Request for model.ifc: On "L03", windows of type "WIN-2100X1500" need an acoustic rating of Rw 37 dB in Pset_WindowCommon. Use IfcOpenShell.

First a look at what the model holds.

```python
import ifcopenshell
import ifcopenshell.util.element

model = ifcopenshell.open("model.ifc")
print(model.schema)
storey = next(s for s in model.by_type("IfcBuildingStorey") if s.Name == "L03")
windows = [e for e in ifcopenshell.util.element.get_decomposition(storey) if e.is_a("IfcWindow")]
seen = {}
for e in windows:
    element_type = ifcopenshell.util.element.get_type(e)
    key = (element_type.Name if element_type != e and element_type else None, ifcopenshell.util.element.get_pset(e, "Pset_WindowCommon", "AcousticRating"))
    seen[key] = seen.get(key, 0) + 1
for (name, value), count in sorted(seen.items(), key=str):
    print(count, "x", name, "|", value)
```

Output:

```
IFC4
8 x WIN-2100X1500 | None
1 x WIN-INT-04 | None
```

```python
import ifcopenshell
import ifcopenshell.api.pset
import ifcopenshell.util.element

model = ifcopenshell.open("model.ifc")

storey = next(s for s in model.by_type("IfcBuildingStorey") if s.Name == "L03")
windows = [e for e in ifcopenshell.util.element.get_decomposition(storey) if e.is_a("IfcWindow")]

count = 0
for e in windows:
    element_type = ifcopenshell.util.element.get_type(e)
    if element_type in (None, e) or element_type.Name != "WIN-2100X1500":
        continue
    # add_pset returns the element's existing set when there is one.
    pset = ifcopenshell.api.pset.add_pset(model, product=e, name="Pset_WindowCommon")
    ifcopenshell.api.pset.edit_pset(model, pset=pset, properties={"AcousticRating": "Rw 37 dB"})
    count += 1

print(count, "windows updated")

model.write("model_v2.ifc")
```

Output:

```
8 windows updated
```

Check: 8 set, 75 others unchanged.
